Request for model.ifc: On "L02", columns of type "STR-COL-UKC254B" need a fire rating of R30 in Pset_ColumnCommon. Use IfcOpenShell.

First a look at what the model holds.

```python
import ifcopenshell
import ifcopenshell.util.element

model = ifcopenshell.open("model.ifc")
print(model.schema)
storey = next(s for s in model.by_type("IfcBuildingStorey") if s.Name == "L02")
columns = [e for e in ifcopenshell.util.element.get_decomposition(storey) if e.is_a("IfcColumn")]
seen = {}
for e in columns:
    element_type = ifcopenshell.util.element.get_type(e)
    key = (element_type.Name if element_type != e and element_type else None, ifcopenshell.util.element.get_pset(e, "Pset_ColumnCommon", "FireRating"))
    seen[key] = seen.get(key, 0) + 1
for (name, value), count in sorted(seen.items(), key=str):
    print(count, "x", name, "|", value)
```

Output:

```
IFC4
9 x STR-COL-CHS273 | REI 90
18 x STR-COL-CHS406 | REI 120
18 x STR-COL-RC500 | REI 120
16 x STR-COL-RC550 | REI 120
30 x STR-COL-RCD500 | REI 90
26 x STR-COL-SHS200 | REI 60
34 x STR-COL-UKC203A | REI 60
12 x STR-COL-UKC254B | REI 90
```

```python
import ifcopenshell
import ifcopenshell.api.pset
import ifcopenshell.util.element

model = ifcopenshell.open("model.ifc")

storey = next(s for s in model.by_type("IfcBuildingStorey") if s.Name == "L02")
columns = [e for e in ifcopenshell.util.element.get_decomposition(storey) if e.is_a("IfcColumn")]

count = 0
for e in columns:
    element_type = ifcopenshell.util.element.get_type(e)
    if element_type in (None, e) or element_type.Name != "STR-COL-UKC254B":
        continue
    # add_pset returns the element's existing set when there is one.
    pset = ifcopenshell.api.pset.add_pset(model, product=e, name="Pset_ColumnCommon")
    ifcopenshell.api.pset.edit_pset(model, pset=pset, properties={"FireRating": "R30"})
    count += 1

print(count, "columns updated")

model.write("model_v2.ifc")
```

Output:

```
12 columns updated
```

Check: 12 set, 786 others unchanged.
